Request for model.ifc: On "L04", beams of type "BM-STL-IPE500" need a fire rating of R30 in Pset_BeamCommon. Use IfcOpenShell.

First a look at what the model holds.

```python
import ifcopenshell
import ifcopenshell.util.element

model = ifcopenshell.open("model.ifc")
print(model.schema)
storey = next(s for s in model.by_type("IfcBuildingStorey") if s.Name == "L04")
beams = [e for e in ifcopenshell.util.element.get_decomposition(storey) if e.is_a("IfcBeam")]
seen = {}
for e in beams:
    element_type = ifcopenshell.util.element.get_type(e)
    key = (element_type.Name if element_type != e and element_type else None, ifcopenshell.util.element.get_pset(e, "Pset_BeamCommon", "FireRating"))
    seen[key] = seen.get(key, 0) + 1
for (name, value), count in sorted(seen.items(), key=str):
    print(count, "x", name, "|", value)
```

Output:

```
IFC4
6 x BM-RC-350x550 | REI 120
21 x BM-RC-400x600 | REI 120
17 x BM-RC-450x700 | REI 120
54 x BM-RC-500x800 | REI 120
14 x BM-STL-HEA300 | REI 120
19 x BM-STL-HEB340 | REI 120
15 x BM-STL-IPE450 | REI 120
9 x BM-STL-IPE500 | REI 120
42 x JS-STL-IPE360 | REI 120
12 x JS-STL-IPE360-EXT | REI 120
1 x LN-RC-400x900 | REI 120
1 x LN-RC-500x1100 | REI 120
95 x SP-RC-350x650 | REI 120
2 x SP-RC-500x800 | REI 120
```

```python
import ifcopenshell
import ifcopenshell.api.pset
import ifcopenshell.util.element

model = ifcopenshell.open("model.ifc")

storey = next(s for s in model.by_type("IfcBuildingStorey") if s.Name == "L04")
beams = [e for e in ifcopenshell.util.element.get_decomposition(storey) if e.is_a("IfcBeam")]

count = 0
for e in beams:
    element_type = ifcopenshell.util.element.get_type(e)
    if element_type in (None, e) or element_type.Name != "BM-STL-IPE500":
        continue
    # add_pset returns the element's existing set when there is one.
    pset = ifcopenshell.api.pset.add_pset(model, product=e, name="Pset_BeamCommon")
    ifcopenshell.api.pset.edit_pset(model, pset=pset, properties={"FireRating": "R30"})
    count += 1

print(count, "beams updated")

model.write("model-out.ifc")
```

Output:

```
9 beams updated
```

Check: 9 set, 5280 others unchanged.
